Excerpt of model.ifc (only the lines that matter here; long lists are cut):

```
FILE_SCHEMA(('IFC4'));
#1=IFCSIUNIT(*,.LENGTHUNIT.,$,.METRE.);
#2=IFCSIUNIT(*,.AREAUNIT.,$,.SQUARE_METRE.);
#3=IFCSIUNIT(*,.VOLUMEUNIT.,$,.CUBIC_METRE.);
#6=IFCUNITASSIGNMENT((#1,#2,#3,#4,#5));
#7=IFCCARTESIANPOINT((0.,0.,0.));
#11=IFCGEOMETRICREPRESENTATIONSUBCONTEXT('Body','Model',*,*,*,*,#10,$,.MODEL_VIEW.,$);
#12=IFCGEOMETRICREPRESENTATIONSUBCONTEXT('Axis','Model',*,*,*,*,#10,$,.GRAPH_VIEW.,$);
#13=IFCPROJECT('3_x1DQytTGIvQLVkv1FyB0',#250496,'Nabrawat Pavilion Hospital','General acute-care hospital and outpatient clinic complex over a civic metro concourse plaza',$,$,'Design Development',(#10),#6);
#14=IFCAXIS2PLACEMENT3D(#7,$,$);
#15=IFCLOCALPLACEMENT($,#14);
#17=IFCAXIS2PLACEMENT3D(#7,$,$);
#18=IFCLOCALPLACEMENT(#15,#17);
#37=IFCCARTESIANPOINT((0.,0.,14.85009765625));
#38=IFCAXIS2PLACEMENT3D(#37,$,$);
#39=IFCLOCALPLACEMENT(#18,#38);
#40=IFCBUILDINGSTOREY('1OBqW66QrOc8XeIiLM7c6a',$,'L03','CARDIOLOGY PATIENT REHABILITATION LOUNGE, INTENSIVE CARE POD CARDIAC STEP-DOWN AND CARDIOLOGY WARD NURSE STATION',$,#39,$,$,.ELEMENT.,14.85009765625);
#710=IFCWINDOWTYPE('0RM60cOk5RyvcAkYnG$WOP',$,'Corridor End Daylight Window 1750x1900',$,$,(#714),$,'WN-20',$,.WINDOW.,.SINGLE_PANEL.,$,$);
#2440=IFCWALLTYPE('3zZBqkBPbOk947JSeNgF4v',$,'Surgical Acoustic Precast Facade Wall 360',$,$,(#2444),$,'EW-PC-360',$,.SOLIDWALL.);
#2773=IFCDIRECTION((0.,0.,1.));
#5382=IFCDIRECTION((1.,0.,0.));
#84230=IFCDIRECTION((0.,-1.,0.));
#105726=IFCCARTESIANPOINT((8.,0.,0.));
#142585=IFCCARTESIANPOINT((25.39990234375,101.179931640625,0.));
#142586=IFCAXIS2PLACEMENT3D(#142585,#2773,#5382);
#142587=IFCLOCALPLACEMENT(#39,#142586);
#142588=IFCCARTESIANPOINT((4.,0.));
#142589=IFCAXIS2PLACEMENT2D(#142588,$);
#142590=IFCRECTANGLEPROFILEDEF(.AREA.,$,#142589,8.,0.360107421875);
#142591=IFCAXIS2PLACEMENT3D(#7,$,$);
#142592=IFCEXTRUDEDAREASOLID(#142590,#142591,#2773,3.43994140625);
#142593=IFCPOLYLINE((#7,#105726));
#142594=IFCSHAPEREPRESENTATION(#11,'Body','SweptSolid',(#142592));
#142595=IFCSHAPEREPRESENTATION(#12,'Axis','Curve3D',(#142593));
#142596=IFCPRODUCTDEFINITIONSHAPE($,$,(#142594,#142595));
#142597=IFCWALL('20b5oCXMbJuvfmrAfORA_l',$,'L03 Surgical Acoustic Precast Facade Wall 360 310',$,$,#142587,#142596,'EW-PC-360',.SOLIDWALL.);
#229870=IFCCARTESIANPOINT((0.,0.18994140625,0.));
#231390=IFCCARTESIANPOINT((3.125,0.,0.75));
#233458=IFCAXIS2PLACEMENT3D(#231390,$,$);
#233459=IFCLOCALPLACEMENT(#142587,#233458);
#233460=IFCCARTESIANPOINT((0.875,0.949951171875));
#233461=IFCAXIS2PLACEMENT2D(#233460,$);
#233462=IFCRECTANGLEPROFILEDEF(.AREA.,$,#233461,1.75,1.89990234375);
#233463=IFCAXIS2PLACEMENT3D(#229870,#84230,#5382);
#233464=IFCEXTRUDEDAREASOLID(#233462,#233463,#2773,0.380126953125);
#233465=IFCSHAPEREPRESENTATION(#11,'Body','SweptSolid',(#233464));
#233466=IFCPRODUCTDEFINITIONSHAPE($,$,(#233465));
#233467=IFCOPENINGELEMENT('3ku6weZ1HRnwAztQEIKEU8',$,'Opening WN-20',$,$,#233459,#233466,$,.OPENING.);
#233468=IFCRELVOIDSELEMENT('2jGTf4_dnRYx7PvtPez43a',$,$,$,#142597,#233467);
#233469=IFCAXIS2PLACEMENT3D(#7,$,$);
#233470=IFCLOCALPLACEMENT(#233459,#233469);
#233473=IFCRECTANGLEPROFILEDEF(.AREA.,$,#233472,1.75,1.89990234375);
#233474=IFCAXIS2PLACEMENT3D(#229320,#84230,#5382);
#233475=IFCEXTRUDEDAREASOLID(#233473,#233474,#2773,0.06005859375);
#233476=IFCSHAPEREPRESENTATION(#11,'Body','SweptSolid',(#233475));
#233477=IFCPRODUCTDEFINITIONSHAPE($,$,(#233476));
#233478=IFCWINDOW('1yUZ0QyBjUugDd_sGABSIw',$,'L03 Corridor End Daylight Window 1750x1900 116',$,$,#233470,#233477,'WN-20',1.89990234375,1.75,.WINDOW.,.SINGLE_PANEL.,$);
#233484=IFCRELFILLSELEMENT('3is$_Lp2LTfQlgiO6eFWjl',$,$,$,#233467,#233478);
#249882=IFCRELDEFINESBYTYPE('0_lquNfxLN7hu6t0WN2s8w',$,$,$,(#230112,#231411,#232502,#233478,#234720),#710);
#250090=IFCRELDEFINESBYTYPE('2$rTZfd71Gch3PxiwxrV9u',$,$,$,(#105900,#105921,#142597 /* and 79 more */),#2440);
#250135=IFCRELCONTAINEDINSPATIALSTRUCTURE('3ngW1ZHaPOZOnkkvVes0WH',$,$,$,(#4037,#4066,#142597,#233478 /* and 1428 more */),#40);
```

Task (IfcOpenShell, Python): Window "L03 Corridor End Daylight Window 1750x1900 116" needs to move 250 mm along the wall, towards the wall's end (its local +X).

```python
import ifcopenshell
import ifcopenshell.api.geometry
import ifcopenshell.util.placement
import ifcopenshell.util.unit

model = ifcopenshell.open("model.ifc")
unit_scale = ifcopenshell.util.unit.calculate_unit_scale(model)

window = model.by_guid("1yUZ0QyBjUugDd_sGABSIw")
opening = window.FillsVoids[0].RelatingOpeningElement
wall = opening.VoidsElements[0].RelatingBuildingElement

wall_matrix = ifcopenshell.util.placement.get_local_placement(wall.ObjectPlacement)
shift = wall_matrix[:3, 0] * 0.25 / unit_scale
before = ifcopenshell.util.placement.get_local_placement(window.ObjectPlacement)[:3, 3].copy()

# The window is placed relative to its opening, so it follows when the opening moves.
matrix = ifcopenshell.util.placement.get_local_placement(opening.ObjectPlacement)
matrix[:3, 3] += shift
ifcopenshell.api.geometry.edit_object_placement(
    model, product=opening, matrix=matrix, is_si=False, should_transform_children=True
)

after = ifcopenshell.util.placement.get_local_placement(window.ObjectPlacement)[:3, 3]
print("window moved by", (after - before).round(3) + 0.0)

model.write("model_updated.ifc")
```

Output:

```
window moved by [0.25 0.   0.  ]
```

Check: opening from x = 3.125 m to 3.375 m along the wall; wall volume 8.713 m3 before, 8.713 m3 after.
